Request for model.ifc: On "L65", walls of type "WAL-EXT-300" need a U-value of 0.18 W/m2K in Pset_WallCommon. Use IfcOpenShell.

First a look at what the model holds.

```python
import ifcopenshell
import ifcopenshell.util.element

model = ifcopenshell.open("model.ifc")
print(model.schema)
storey = next(s for s in model.by_type("IfcBuildingStorey") if s.Name == "L65")
walls = [e for e in ifcopenshell.util.element.get_decomposition(storey) if e.is_a("IfcWall")]
seen = {}
for e in walls:
    element_type = ifcopenshell.util.element.get_type(e)
    key = (element_type.Name if element_type != e and element_type else None, ifcopenshell.util.element.get_pset(e, "Pset_WallCommon", "ThermalTransmittance"))
    seen[key] = seen.get(key, 0) + 1
for (name, value), count in sorted(seen.items(), key=str):
    print(count, "x", name, "|", value)
```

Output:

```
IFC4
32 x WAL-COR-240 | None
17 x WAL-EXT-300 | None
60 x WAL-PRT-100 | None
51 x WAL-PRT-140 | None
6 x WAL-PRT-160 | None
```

```python
import ifcopenshell
import ifcopenshell.api.pset
import ifcopenshell.util.element

model = ifcopenshell.open("model.ifc")

storey = next(s for s in model.by_type("IfcBuildingStorey") if s.Name == "L65")
walls = [e for e in ifcopenshell.util.element.get_decomposition(storey) if e.is_a("IfcWall")]

count = 0
for e in walls:
    element_type = ifcopenshell.util.element.get_type(e)
    if element_type in (None, e) or element_type.Name != "WAL-EXT-300":
        continue
    found = ifcopenshell.util.element.get_pset(e, "Pset_WallCommon", should_inherit=False)
    if found:
        pset = model.by_id(found["id"])
        if len(ifcopenshell.util.element.get_elements_by_pset(pset)) > 1:
            pset = ifcopenshell.api.pset.unshare_pset(model, products=[e], pset=pset)[0]
    else:
        pset = ifcopenshell.api.pset.add_pset(model, product=e, name="Pset_WallCommon")
    ifcopenshell.api.pset.edit_pset(model, pset=pset, properties={"ThermalTransmittance": 0.18})
    count += 1

print(count, "walls updated")

model.write("model_edited.ifc")
```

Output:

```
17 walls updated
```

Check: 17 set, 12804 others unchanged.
